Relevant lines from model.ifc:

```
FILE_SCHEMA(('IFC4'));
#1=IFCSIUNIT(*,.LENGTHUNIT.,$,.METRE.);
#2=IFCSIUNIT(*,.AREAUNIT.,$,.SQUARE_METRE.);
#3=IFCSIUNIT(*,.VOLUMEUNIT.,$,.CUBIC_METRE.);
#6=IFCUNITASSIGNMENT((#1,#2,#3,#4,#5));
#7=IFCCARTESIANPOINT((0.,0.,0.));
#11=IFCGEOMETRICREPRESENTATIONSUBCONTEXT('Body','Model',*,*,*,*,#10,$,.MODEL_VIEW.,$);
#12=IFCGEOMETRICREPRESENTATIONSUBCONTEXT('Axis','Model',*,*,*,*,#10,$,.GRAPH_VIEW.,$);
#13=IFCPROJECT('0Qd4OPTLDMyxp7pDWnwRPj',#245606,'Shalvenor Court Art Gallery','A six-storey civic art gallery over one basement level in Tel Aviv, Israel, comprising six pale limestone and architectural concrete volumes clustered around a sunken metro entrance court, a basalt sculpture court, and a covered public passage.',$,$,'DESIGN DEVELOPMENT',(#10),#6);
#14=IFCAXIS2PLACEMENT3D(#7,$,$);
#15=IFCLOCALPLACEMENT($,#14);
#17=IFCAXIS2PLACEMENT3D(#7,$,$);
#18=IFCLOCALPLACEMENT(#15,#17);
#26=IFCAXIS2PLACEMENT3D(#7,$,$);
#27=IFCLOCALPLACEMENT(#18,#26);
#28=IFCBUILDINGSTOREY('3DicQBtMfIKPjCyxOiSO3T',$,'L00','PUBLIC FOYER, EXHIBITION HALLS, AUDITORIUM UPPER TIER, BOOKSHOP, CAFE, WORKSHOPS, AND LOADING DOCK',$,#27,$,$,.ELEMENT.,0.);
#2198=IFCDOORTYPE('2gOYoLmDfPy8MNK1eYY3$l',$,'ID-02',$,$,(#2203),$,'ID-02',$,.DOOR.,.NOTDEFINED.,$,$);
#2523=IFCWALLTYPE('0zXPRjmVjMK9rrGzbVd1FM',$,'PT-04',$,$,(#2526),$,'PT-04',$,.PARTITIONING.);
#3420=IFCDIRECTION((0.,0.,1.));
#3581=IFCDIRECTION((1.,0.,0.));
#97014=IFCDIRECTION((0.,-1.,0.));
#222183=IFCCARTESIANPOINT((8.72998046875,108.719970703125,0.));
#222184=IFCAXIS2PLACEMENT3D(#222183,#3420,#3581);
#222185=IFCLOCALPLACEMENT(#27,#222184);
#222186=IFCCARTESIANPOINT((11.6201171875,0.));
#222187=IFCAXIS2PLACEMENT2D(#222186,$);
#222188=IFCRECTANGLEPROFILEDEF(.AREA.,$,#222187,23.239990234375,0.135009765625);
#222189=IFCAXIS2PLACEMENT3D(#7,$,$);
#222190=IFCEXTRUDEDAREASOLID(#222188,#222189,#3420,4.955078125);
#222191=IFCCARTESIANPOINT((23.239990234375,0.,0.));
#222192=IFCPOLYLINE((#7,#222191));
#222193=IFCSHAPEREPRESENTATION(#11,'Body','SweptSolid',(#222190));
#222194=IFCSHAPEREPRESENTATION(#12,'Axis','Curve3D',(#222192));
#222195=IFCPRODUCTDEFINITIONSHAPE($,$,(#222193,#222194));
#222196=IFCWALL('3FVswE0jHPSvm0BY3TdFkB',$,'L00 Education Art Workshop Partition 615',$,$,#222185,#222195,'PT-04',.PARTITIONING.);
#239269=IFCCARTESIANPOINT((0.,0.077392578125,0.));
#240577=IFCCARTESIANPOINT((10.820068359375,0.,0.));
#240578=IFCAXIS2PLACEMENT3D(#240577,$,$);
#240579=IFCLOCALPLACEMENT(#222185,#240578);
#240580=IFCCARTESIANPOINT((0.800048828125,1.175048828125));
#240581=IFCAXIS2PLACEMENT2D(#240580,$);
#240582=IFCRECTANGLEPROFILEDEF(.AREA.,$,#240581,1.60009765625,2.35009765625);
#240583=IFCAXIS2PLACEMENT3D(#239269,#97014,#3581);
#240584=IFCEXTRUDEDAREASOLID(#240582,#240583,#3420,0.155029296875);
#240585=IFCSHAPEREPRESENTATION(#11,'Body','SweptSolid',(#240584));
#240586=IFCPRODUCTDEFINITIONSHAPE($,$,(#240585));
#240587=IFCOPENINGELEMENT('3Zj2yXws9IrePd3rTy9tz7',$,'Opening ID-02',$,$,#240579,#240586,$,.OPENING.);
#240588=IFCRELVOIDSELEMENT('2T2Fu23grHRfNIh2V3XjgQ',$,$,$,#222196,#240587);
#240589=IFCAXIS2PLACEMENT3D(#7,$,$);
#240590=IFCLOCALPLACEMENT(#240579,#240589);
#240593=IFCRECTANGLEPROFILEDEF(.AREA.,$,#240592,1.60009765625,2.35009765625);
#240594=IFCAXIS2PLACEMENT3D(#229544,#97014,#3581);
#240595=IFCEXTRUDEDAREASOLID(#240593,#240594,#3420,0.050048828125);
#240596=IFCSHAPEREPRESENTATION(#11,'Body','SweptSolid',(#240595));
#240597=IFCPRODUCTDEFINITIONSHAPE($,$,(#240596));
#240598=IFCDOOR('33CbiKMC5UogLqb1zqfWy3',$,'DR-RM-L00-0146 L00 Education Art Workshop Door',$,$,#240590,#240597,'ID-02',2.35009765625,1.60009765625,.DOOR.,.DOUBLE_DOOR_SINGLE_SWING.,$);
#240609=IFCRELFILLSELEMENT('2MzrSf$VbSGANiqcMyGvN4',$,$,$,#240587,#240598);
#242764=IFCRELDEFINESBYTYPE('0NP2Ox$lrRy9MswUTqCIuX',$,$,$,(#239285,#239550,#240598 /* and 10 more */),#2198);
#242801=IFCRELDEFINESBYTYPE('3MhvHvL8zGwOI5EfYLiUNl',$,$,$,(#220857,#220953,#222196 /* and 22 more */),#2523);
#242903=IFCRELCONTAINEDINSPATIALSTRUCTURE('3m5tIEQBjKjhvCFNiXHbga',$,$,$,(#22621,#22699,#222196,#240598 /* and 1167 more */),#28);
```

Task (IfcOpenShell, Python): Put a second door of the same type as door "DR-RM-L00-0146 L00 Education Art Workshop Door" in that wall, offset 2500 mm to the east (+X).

```python
import ifcopenshell
import ifcopenshell.api.feature
import ifcopenshell.api.geometry
import ifcopenshell.api.root
import ifcopenshell.geom
import ifcopenshell.util.element
import ifcopenshell.util.placement
import ifcopenshell.util.shape
import ifcopenshell.util.unit

model = ifcopenshell.open("model.ifc")
unit_scale = ifcopenshell.util.unit.calculate_unit_scale(model)
settings = ifcopenshell.geom.settings()


def volume(element):
    """Net volume in cubic metres, openings subtracted."""
    shape = ifcopenshell.geom.create_shape(settings, element)
    return ifcopenshell.util.shape.get_volume(shape.geometry)


door = model.by_guid("33CbiKMC5UogLqb1zqfWy3")
opening = door.FillsVoids[0].RelatingOpeningElement
wall = opening.VoidsElements[0].RelatingBuildingElement
before = volume(wall)
shift = ifcopenshell.util.placement.get_local_placement(wall.ObjectPlacement)[:3, 0] * 2.5 / unit_scale

# copy_class copies the void relationship, type, container and properties, but no geometry.
new_opening = ifcopenshell.api.root.copy_class(model, product=opening)
new_opening.Representation = ifcopenshell.util.element.copy_deep(
    model, opening.Representation, exclude=["IfcGeometricRepresentationContext", "IfcRepresentationMap"]
)
new_door = ifcopenshell.api.root.copy_class(model, product=door)
new_door.Representation = ifcopenshell.util.element.copy_deep(
    model, door.Representation, exclude=["IfcGeometricRepresentationContext", "IfcRepresentationMap"]
)
new_door.Tag = None
ifcopenshell.api.feature.add_filling(model, opening=new_opening, element=new_door)

for old, new in ((opening, new_opening), (door, new_door)):
    matrix = ifcopenshell.util.placement.get_local_placement(old.ObjectPlacement)
    matrix[:3, 3] += shift
    ifcopenshell.api.geometry.edit_object_placement(model, product=new, matrix=matrix, is_si=False)

after = volume(wall)

print(f"wall volume {before:.3f} -> {after:.3f} m3")

model.write("model-out.ifc")
```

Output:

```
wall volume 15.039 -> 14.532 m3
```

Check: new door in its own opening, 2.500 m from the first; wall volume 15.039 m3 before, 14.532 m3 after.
